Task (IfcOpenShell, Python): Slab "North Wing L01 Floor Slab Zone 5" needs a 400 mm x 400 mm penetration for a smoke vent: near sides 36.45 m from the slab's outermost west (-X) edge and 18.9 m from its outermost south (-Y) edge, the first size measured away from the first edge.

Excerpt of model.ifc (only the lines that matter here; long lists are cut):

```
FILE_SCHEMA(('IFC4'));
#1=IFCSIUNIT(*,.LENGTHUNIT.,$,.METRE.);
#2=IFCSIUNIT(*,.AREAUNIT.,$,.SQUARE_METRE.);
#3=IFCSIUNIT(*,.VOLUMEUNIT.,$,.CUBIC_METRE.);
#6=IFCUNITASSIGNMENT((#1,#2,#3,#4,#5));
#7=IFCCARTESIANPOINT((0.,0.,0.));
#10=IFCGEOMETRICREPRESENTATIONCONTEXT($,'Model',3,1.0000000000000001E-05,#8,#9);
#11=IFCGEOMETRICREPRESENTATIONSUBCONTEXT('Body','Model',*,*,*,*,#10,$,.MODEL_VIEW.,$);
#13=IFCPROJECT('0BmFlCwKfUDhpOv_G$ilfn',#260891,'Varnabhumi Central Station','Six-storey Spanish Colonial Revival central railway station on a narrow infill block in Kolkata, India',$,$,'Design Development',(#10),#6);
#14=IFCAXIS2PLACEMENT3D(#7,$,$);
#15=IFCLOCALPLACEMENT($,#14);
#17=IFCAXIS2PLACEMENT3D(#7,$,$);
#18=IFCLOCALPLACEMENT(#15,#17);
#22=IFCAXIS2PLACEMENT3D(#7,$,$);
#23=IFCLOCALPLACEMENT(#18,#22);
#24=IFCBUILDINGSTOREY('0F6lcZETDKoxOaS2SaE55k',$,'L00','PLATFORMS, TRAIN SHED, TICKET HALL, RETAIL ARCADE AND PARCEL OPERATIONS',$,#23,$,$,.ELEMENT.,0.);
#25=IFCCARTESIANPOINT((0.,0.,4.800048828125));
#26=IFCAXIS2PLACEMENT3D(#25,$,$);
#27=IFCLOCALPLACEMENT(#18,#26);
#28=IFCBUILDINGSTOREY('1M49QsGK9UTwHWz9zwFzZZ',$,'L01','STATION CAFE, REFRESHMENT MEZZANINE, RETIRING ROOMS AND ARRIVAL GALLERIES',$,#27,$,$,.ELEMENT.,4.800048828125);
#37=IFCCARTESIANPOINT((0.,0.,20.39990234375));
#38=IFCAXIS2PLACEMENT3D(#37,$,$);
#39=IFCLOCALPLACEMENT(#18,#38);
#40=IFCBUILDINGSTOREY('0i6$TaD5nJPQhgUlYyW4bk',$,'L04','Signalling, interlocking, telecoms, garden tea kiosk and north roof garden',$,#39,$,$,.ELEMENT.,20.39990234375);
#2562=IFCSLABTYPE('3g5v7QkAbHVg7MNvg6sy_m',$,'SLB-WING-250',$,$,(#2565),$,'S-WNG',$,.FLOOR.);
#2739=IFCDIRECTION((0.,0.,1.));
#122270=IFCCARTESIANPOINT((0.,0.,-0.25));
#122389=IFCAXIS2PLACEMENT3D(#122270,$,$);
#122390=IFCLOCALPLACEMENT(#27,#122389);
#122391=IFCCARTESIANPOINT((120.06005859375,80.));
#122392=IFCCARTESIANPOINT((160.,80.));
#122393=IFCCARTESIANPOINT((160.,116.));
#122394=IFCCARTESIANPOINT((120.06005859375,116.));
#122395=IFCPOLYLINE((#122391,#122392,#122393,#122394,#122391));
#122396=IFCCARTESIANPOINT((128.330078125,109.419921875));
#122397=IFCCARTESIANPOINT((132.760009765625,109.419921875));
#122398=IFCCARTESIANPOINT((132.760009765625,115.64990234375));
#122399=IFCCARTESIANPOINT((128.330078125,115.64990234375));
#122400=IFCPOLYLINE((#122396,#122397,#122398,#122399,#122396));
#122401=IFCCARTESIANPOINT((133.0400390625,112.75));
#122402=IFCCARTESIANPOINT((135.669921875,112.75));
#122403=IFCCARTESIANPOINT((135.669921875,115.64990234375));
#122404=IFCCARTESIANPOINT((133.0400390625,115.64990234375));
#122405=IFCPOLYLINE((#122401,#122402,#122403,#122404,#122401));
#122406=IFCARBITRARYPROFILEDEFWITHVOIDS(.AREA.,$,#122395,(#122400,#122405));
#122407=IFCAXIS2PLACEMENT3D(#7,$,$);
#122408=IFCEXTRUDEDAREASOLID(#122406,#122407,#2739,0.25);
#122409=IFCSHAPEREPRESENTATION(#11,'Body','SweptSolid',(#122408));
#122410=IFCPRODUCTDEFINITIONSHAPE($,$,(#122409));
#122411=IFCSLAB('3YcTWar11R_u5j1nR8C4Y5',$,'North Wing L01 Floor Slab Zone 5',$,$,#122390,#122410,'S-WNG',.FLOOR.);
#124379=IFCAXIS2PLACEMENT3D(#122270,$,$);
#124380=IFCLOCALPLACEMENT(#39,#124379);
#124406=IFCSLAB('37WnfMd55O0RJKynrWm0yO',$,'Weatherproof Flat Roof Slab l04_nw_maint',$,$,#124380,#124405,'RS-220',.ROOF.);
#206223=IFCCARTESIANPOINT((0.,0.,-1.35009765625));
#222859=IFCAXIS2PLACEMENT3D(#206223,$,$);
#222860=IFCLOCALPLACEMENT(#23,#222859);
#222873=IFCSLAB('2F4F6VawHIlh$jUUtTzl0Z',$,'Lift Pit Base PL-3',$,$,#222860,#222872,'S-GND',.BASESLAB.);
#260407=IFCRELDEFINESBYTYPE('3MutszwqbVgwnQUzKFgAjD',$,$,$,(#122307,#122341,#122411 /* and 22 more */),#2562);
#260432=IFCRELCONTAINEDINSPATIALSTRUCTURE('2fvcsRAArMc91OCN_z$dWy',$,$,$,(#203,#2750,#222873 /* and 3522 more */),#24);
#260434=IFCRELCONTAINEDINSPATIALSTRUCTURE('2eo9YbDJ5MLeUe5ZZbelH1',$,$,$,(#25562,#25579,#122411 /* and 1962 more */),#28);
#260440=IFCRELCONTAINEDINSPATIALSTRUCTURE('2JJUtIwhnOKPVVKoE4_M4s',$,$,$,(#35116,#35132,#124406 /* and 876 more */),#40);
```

```python
import numpy as np
import ifcopenshell
import ifcopenshell.api.feature
import ifcopenshell.api.geometry
import ifcopenshell.api.root
import ifcopenshell.geom
import ifcopenshell.util.placement
import ifcopenshell.util.representation
import ifcopenshell.util.shape
import ifcopenshell.util.unit

model = ifcopenshell.open("model.ifc")
unit_scale = ifcopenshell.util.unit.calculate_unit_scale(model)
settings = ifcopenshell.geom.settings()


def volume(element):
    """Net volume in cubic metres, openings subtracted."""
    shape = ifcopenshell.geom.create_shape(settings, element)
    return ifcopenshell.util.shape.get_volume(shape.geometry)


slab = model.by_id(122411)
before = volume(slab)

# Extent in the slab's own axes, in metres. The edges named are its -X and -Y sides.
slab_shape = ifcopenshell.geom.create_shape(settings, slab)
vertices = ifcopenshell.util.shape.get_vertices(slab_shape.geometry)
x_min, y_min, bottom = vertices.min(axis=0)
top = vertices[:, 2].max()

opening = ifcopenshell.api.root.create_entity(model, ifc_class="IfcOpeningElement", name="Smoke vent opening", predefined_type="OPENING")
context = ifcopenshell.util.representation.get_context(model, "Model", "Body", "MODEL_VIEW")
width, depth = 0.4, 0.4
outline = [(0.0, 0.0), (width, 0.0), (width, depth), (0.0, depth), (0.0, 0.0)]
# Overshoot both faces by 50 mm so the cut is clean.
shape = ifcopenshell.api.geometry.add_slab_representation(
    model, context=context, depth=top - bottom + 0.1, polyline=outline
)
ifcopenshell.api.geometry.assign_representation(model, product=opening, representation=shape)

matrix = ifcopenshell.util.placement.get_local_placement(slab.ObjectPlacement)
matrix[:, 3] = matrix @ np.append(np.array([x_min + 36.45, y_min + 18.9, bottom - 0.05]) / unit_scale, 1.0)
ifcopenshell.api.geometry.edit_object_placement(model, product=opening, matrix=matrix, is_si=False)
ifcopenshell.api.feature.add_feature(model, feature=opening, element=slab)

after = volume(slab)

print(f"slab volume {before:.3f} -> {after:.3f} m3")

model.write("model_v2.ifc")
```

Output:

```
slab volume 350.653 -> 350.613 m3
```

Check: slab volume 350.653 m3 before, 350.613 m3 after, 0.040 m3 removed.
